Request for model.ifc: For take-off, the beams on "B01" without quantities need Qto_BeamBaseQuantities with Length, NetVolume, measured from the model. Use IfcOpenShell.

First a look at what the model holds.

```python
import ifcopenshell
import ifcopenshell.util.element
import ifcopenshell.util.unit

model = ifcopenshell.open("model.ifc")
print(model.schema)
for unit_type in ("LENGTHUNIT", "AREAUNIT", "VOLUMEUNIT"):
    print(unit_type, ifcopenshell.util.unit.calculate_unit_scale(model, unit_type))
storey = next(s for s in model.by_type("IfcBuildingStorey") if s.Name == "B01")
beams = [e for e in ifcopenshell.util.element.get_decomposition(storey) if e.is_a("IfcBeam")]
for e in sorted(beams, key=lambda e: e.id()):
    print(e.id(), e.is_a(), e.Name, list(ifcopenshell.util.element.get_psets(e, qtos_only=True)), sep=" | ")
```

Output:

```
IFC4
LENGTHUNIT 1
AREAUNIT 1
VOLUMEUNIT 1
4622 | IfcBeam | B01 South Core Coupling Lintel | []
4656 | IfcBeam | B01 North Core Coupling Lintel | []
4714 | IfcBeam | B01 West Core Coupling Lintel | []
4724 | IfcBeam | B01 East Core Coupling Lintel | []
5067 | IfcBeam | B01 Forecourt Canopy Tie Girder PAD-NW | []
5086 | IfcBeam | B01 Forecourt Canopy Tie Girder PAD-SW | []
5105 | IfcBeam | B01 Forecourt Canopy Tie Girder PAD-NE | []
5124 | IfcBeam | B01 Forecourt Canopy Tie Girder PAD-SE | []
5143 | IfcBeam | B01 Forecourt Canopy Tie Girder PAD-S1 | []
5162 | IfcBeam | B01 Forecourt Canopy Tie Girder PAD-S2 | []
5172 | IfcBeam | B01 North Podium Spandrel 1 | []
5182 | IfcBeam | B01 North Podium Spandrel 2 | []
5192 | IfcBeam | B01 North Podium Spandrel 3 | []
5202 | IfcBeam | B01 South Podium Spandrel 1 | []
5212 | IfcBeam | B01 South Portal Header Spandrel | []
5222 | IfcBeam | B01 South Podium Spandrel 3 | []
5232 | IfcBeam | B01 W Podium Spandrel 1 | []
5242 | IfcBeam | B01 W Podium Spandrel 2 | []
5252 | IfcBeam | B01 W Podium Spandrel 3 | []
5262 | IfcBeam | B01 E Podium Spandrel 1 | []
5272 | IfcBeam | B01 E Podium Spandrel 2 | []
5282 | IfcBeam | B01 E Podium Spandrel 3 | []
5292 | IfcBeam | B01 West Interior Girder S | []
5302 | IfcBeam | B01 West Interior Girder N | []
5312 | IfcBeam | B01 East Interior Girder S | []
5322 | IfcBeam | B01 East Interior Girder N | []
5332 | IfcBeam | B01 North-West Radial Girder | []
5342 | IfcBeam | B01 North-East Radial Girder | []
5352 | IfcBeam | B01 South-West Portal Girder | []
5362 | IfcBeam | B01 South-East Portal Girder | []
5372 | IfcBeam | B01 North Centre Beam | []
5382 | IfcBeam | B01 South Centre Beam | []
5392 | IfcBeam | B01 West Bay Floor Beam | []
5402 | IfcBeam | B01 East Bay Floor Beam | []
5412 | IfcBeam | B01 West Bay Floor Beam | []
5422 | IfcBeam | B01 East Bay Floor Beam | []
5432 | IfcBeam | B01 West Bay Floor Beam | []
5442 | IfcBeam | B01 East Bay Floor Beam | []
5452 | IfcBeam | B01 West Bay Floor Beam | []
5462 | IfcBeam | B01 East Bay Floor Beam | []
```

```python
import ifcopenshell
import ifcopenshell.api.pset
import ifcopenshell.geom
import ifcopenshell.util.element
import ifcopenshell.util.shape
import ifcopenshell.util.unit

model = ifcopenshell.open("model.ifc")
unit_scale = ifcopenshell.util.unit.calculate_unit_scale(model)
volume_scale = ifcopenshell.util.unit.calculate_unit_scale(model, "VOLUMEUNIT")
settings = ifcopenshell.geom.settings()

storey = next(s for s in model.by_type("IfcBuildingStorey") if s.Name == "B01")
beams = [e for e in ifcopenshell.util.element.get_decomposition(storey) if e.is_a("IfcBeam")]

for e in sorted(beams, key=lambda e: e.id()):
    if ifcopenshell.util.element.get_psets(e, qtos_only=True, should_inherit=False):
        continue
    # Geometry comes back in metres, in the element's own axes.
    shape = ifcopenshell.geom.create_shape(settings, e)
    values = {
        "Length": ifcopenshell.util.shape.get_max_xyz(shape.geometry) / unit_scale,
        "NetVolume": ifcopenshell.util.shape.get_volume(shape.geometry) / volume_scale,
    }
    qto = ifcopenshell.api.pset.add_qto(model, product=e, name="Qto_BeamBaseQuantities")
    ifcopenshell.api.pset.edit_qto(model, qto=qto, properties=values)
    print(e.id(), {k: round(v, 3) for k, v in values.items()})

model.write("model-out.ifc")
```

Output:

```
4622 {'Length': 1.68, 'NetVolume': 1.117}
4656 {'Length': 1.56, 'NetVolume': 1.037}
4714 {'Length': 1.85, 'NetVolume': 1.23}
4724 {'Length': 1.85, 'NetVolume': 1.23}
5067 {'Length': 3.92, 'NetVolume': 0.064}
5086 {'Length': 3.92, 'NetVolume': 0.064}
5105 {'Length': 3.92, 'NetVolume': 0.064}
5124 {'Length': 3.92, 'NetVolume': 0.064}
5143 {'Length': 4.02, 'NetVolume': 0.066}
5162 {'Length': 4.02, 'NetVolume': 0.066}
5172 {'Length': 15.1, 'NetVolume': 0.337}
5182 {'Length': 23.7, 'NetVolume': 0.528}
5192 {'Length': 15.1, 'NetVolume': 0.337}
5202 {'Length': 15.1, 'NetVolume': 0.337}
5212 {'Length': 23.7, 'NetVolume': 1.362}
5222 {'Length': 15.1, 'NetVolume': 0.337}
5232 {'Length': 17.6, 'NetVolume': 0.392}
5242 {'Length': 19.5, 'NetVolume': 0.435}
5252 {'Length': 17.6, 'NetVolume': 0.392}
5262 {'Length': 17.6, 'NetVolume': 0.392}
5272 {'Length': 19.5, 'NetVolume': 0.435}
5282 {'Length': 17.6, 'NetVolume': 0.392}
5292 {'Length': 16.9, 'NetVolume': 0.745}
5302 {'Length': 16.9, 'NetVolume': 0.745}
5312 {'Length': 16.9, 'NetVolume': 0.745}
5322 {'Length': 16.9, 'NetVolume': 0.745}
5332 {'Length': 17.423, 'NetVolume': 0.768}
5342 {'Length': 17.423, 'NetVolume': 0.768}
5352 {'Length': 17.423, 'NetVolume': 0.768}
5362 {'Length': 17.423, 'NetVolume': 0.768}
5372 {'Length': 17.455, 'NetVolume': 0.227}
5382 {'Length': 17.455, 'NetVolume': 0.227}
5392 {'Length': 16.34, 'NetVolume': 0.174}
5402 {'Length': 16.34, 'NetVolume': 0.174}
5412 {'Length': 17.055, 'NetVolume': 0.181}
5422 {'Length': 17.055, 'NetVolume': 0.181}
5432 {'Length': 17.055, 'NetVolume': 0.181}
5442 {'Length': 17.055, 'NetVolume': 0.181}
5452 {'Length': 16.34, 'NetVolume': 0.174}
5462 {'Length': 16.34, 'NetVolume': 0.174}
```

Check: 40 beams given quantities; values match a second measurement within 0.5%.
